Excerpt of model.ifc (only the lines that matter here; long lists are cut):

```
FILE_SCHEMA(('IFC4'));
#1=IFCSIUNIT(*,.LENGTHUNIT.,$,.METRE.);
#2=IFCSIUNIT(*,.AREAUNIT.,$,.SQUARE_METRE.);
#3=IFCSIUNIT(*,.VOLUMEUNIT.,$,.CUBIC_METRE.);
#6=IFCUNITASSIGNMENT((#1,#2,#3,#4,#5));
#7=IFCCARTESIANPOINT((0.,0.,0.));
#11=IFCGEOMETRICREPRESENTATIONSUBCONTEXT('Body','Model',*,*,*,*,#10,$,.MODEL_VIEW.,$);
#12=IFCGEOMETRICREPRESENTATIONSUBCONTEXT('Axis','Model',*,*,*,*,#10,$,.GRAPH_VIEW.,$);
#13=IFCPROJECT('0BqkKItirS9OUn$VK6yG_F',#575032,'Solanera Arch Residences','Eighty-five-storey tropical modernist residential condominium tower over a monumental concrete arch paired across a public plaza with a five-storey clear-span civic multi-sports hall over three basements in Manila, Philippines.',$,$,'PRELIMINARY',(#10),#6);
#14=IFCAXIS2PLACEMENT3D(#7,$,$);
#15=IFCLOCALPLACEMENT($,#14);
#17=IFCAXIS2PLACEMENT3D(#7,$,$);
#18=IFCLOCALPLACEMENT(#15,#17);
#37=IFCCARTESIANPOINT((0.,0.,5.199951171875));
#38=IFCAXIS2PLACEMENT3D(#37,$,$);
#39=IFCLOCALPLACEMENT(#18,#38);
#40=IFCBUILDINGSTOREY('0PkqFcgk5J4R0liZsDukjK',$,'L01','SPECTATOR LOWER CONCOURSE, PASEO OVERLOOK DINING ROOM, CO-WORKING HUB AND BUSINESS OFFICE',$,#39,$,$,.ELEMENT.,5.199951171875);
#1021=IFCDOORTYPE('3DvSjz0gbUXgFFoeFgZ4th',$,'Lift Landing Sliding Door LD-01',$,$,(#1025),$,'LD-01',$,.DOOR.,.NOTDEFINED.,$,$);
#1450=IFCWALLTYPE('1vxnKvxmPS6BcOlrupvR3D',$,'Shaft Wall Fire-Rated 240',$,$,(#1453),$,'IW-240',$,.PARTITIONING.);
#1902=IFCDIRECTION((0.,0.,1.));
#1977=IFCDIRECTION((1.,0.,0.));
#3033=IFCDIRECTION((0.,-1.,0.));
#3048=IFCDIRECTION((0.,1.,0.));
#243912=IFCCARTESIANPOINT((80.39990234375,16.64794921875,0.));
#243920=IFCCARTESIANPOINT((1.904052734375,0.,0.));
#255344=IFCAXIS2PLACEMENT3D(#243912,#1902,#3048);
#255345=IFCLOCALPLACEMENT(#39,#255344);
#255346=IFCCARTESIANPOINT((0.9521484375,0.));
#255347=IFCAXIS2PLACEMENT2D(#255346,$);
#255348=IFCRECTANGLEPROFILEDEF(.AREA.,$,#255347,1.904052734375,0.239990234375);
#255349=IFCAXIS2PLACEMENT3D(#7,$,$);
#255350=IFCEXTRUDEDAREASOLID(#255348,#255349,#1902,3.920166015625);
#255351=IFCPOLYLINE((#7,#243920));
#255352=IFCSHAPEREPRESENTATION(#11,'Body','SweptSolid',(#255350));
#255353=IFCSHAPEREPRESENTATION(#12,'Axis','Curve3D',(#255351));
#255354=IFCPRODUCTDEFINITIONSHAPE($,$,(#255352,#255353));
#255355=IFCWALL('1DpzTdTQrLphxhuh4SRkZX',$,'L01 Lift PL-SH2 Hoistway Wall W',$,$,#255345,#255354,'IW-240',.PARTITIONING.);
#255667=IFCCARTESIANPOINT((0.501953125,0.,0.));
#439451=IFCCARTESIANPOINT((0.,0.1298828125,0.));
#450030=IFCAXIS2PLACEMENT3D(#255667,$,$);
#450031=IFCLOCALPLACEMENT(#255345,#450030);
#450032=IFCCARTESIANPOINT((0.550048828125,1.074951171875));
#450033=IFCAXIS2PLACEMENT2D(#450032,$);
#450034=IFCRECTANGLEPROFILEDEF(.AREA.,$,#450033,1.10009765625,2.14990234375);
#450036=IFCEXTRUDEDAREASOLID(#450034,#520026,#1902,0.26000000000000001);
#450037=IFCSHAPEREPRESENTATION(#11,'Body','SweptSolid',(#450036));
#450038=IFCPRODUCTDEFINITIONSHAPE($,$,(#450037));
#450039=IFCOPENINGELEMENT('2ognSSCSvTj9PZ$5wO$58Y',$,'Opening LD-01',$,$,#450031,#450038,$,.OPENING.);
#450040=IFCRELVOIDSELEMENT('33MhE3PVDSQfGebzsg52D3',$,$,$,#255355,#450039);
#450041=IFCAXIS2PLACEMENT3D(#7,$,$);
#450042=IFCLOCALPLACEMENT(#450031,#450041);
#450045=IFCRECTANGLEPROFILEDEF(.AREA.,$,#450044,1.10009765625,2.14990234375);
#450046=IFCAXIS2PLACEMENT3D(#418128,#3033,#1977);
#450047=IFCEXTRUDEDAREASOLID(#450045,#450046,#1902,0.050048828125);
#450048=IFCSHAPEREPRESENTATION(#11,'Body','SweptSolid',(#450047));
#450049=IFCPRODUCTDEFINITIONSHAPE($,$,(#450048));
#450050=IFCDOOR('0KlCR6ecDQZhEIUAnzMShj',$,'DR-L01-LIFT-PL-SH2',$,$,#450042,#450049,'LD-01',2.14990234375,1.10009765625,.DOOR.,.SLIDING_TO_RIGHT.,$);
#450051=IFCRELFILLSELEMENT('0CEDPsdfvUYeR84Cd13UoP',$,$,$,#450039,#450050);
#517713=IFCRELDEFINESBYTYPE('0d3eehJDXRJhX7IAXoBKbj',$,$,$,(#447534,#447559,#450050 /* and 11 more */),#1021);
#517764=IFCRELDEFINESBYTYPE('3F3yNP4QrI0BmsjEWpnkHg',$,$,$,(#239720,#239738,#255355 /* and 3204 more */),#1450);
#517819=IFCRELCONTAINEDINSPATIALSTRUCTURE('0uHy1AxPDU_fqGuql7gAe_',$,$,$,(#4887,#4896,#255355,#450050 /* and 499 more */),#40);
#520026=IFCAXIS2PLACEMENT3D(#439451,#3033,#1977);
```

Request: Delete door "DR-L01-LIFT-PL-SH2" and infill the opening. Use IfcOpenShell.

```python
import ifcopenshell
import ifcopenshell.api.feature
import ifcopenshell.api.root
import ifcopenshell.geom
import ifcopenshell.util.shape

model = ifcopenshell.open("model.ifc")
settings = ifcopenshell.geom.settings()


def volume(element):
    """Net volume in cubic metres, openings subtracted."""
    shape = ifcopenshell.geom.create_shape(settings, element)
    return ifcopenshell.util.shape.get_volume(shape.geometry)


door = model.by_guid("0KlCR6ecDQZhEIUAnzMShj")
opening = door.FillsVoids[0].RelatingOpeningElement
wall = opening.VoidsElements[0].RelatingBuildingElement
before = volume(wall)

ifcopenshell.api.root.remove_product(model, product=door)
ifcopenshell.api.feature.remove_feature(model, feature=opening)

after = volume(wall)

print(f"wall volume {before:.3f} -> {after:.3f} m3")

model.write("model_rev.ifc")
```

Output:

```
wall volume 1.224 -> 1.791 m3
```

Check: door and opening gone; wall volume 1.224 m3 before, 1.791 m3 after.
